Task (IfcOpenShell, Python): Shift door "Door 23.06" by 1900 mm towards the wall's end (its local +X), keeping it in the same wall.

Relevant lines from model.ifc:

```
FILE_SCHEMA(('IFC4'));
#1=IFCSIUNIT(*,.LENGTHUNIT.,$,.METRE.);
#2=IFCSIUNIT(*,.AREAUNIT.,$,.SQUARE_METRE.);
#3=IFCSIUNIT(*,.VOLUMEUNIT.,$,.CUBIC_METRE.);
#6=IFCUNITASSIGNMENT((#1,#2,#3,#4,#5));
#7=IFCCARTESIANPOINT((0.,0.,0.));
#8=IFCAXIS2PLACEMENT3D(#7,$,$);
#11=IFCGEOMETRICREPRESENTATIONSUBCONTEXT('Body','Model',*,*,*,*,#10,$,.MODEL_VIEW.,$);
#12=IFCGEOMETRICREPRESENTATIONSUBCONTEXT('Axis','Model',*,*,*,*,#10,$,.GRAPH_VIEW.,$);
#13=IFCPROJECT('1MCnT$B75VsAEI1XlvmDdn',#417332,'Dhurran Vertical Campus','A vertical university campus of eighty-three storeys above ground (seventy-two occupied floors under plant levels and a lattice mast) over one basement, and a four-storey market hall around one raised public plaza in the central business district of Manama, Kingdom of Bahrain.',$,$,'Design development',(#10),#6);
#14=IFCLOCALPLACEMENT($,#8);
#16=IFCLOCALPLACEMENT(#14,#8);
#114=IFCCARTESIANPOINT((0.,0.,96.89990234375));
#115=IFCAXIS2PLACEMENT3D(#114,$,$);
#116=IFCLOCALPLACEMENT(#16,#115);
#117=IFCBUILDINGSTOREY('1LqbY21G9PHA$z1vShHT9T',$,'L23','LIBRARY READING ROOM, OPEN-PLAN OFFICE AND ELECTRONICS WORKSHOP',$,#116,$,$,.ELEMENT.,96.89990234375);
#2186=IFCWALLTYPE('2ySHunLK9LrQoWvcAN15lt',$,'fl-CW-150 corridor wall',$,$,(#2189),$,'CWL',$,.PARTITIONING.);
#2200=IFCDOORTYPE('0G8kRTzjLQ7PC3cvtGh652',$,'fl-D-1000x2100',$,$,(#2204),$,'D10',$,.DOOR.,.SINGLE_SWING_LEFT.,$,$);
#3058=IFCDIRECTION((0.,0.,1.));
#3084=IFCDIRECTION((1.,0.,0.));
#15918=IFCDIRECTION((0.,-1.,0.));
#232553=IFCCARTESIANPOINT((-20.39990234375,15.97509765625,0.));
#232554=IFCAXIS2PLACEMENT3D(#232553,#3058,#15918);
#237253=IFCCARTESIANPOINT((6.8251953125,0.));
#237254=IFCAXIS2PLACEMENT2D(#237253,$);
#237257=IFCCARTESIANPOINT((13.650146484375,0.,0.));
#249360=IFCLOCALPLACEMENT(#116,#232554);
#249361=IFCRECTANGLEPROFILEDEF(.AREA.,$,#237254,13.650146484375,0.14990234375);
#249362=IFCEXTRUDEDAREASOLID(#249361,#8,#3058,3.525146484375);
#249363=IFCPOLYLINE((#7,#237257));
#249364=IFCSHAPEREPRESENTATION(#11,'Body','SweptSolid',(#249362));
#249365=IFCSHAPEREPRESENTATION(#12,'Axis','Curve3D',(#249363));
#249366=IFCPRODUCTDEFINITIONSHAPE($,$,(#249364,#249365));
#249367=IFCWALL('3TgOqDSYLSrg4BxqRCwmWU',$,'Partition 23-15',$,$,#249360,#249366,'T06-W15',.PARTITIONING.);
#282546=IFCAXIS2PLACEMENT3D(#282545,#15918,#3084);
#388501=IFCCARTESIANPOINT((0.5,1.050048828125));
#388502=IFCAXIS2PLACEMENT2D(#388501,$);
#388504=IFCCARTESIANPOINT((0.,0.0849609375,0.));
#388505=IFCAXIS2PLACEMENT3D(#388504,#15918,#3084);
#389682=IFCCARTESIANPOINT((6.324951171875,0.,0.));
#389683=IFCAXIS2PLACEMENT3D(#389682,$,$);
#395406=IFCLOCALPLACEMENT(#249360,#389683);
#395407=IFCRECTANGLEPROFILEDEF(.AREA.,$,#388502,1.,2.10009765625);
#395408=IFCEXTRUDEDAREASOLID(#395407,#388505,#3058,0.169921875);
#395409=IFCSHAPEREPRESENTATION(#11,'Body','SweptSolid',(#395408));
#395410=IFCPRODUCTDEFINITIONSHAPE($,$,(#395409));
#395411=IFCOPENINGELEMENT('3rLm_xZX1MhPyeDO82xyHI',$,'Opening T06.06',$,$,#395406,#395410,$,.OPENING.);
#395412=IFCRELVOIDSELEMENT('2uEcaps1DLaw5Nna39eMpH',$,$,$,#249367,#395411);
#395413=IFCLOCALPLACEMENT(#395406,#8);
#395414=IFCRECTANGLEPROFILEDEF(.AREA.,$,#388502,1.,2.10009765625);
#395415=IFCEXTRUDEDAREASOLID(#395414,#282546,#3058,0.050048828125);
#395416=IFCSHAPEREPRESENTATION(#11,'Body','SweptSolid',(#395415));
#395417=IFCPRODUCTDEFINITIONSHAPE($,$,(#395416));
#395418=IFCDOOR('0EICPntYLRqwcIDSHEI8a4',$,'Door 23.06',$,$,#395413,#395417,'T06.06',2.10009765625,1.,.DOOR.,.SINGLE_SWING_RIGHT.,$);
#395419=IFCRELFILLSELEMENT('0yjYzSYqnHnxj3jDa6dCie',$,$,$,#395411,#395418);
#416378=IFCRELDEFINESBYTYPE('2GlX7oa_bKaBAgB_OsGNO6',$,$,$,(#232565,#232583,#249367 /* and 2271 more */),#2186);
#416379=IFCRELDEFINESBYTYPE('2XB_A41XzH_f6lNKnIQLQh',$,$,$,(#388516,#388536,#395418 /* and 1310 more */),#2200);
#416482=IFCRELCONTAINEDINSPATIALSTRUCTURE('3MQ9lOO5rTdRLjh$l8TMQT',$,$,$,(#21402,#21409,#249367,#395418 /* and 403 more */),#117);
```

```python
import ifcopenshell
import ifcopenshell.api.geometry
import ifcopenshell.util.placement
import ifcopenshell.util.unit

model = ifcopenshell.open("model.ifc")
unit_scale = ifcopenshell.util.unit.calculate_unit_scale(model)

door = model.by_guid("0EICPntYLRqwcIDSHEI8a4")
opening = door.FillsVoids[0].RelatingOpeningElement
wall = opening.VoidsElements[0].RelatingBuildingElement

wall_matrix = ifcopenshell.util.placement.get_local_placement(wall.ObjectPlacement)
shift = wall_matrix[:3, 0] * 1.9 / unit_scale
before = ifcopenshell.util.placement.get_local_placement(door.ObjectPlacement)[:3, 3].copy()

# The door is placed relative to its opening, so it follows when the opening moves.
matrix = ifcopenshell.util.placement.get_local_placement(opening.ObjectPlacement)
matrix[:3, 3] += shift
ifcopenshell.api.geometry.edit_object_placement(
    model, product=opening, matrix=matrix, is_si=False, should_transform_children=True
)

after = ifcopenshell.util.placement.get_local_placement(door.ObjectPlacement)[:3, 3]
print("door moved by", (after - before).round(3) + 0.0)

model.write("model_v2.ifc")
```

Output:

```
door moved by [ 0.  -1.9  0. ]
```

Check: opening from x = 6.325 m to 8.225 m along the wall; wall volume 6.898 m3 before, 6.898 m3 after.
